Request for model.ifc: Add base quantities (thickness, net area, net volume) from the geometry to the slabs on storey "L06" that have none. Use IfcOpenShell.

First a look at what the model holds.

```python
import ifcopenshell
import ifcopenshell.util.element
import ifcopenshell.util.unit

model = ifcopenshell.open("model.ifc")
print(model.schema)
for unit_type in ("LENGTHUNIT", "AREAUNIT", "VOLUMEUNIT"):
    print(unit_type, ifcopenshell.util.unit.calculate_unit_scale(model, unit_type))
storey = next(s for s in model.by_type("IfcBuildingStorey") if s.Name == "L06")
slabs = [e for e in ifcopenshell.util.element.get_decomposition(storey) if e.is_a("IfcSlab")]
for e in sorted(slabs, key=lambda e: e.id()):
    print(e.id(), e.is_a(), e.Name, list(ifcopenshell.util.element.get_psets(e, qtos_only=True)), sep=" | ")
```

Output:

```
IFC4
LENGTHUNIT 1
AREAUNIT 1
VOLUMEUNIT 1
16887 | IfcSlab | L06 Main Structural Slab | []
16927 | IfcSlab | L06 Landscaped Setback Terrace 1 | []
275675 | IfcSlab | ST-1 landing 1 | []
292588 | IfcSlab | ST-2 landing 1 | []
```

```python
import ifcopenshell
import ifcopenshell.api.pset
import ifcopenshell.geom
import ifcopenshell.util.element
import ifcopenshell.util.shape
import ifcopenshell.util.unit

model = ifcopenshell.open("model.ifc")
unit_scale = ifcopenshell.util.unit.calculate_unit_scale(model)
area_scale = ifcopenshell.util.unit.calculate_unit_scale(model, "AREAUNIT")
volume_scale = ifcopenshell.util.unit.calculate_unit_scale(model, "VOLUMEUNIT")
settings = ifcopenshell.geom.settings()

storey = next(s for s in model.by_type("IfcBuildingStorey") if s.Name == "L06")
slabs = [e for e in ifcopenshell.util.element.get_decomposition(storey) if e.is_a("IfcSlab")]

for e in sorted(slabs, key=lambda e: e.id()):
    if ifcopenshell.util.element.get_psets(e, qtos_only=True, should_inherit=False):
        continue
    # Geometry comes back in metres, in the element's own axes.
    shape = ifcopenshell.geom.create_shape(settings, e)
    values = {
        "Width": ifcopenshell.util.shape.get_z(shape.geometry) / unit_scale,
        "NetArea": ifcopenshell.util.shape.get_footprint_area(shape.geometry) / area_scale,
        "NetVolume": ifcopenshell.util.shape.get_volume(shape.geometry) / volume_scale,
    }
    qto = ifcopenshell.api.pset.add_qto(model, product=e, name="Qto_SlabBaseQuantities")
    ifcopenshell.api.pset.edit_qto(model, qto=qto, properties=values)
    print(e.id(), {k: round(v, 3) for k, v in values.items()})

model.write("model_edited.ifc")
```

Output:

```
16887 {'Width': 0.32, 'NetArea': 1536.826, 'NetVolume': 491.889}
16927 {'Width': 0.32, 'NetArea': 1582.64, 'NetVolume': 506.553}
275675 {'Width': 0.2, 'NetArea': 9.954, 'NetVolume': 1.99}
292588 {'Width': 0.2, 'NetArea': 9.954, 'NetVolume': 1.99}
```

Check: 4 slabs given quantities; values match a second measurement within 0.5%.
